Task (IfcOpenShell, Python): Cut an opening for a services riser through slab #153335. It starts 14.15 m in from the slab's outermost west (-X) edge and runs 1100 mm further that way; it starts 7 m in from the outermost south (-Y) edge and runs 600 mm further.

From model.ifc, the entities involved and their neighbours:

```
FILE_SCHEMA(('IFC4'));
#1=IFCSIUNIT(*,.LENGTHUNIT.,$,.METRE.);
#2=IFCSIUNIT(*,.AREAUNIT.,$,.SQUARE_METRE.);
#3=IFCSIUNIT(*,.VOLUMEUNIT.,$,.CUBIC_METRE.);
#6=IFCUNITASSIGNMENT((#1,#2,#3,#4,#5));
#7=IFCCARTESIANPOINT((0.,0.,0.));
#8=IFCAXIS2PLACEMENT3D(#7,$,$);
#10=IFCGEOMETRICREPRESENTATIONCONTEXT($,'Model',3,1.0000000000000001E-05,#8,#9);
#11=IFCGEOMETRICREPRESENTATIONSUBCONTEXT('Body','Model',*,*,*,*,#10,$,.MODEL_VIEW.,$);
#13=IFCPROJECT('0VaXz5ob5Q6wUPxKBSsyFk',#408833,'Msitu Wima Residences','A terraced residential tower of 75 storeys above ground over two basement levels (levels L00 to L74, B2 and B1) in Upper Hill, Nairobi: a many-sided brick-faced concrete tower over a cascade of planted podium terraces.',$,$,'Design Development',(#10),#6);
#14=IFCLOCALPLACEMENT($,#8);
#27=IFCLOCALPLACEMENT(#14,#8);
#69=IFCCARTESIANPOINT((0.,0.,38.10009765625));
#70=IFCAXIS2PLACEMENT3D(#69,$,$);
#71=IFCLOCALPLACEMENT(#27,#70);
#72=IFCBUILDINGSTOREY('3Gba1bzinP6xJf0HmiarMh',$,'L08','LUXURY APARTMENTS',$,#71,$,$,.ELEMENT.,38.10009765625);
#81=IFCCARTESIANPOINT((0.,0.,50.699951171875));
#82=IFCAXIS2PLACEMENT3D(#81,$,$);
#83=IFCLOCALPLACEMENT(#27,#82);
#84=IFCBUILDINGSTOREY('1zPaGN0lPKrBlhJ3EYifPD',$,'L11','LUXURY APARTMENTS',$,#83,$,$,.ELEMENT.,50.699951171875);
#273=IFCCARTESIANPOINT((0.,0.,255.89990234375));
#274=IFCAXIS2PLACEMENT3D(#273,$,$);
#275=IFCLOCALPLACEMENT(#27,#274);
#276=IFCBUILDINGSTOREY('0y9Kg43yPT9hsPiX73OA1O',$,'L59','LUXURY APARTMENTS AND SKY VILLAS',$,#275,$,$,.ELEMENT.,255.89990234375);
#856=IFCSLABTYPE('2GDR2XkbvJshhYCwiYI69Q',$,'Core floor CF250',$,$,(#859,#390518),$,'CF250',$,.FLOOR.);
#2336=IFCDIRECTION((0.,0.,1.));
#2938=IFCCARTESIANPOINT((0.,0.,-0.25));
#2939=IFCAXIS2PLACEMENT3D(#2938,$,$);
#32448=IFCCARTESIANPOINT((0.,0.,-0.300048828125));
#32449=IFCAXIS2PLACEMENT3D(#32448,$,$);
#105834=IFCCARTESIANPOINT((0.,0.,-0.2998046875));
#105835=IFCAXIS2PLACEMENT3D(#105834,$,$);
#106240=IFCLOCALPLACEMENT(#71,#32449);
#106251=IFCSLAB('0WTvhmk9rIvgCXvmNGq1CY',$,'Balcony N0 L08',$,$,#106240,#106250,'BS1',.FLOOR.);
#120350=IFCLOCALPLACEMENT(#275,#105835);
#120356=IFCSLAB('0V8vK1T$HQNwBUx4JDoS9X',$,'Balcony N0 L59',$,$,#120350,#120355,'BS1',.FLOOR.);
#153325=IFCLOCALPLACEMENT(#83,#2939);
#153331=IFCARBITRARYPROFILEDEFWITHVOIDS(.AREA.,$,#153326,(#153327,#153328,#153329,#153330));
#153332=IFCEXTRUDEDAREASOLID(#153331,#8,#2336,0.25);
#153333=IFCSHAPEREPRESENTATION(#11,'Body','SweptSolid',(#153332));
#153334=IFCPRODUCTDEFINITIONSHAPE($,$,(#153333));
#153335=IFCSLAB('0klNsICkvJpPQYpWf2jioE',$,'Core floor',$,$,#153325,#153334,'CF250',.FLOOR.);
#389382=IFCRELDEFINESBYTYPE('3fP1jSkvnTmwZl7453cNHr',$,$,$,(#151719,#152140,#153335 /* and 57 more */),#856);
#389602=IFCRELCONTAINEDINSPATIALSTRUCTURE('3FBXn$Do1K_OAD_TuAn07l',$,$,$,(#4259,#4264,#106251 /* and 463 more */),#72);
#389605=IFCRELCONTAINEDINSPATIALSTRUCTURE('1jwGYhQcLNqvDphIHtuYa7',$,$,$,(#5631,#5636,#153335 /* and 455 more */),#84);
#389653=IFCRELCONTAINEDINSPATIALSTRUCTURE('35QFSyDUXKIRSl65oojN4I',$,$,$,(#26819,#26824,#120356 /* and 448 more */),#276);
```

```python
import numpy as np
import ifcopenshell
import ifcopenshell.api.feature
import ifcopenshell.api.geometry
import ifcopenshell.api.root
import ifcopenshell.geom
import ifcopenshell.util.placement
import ifcopenshell.util.representation
import ifcopenshell.util.shape
import ifcopenshell.util.unit

model = ifcopenshell.open("model.ifc")
unit_scale = ifcopenshell.util.unit.calculate_unit_scale(model)
settings = ifcopenshell.geom.settings()


def volume(element):
    """Net volume in cubic metres, openings subtracted."""
    shape = ifcopenshell.geom.create_shape(settings, element)
    return ifcopenshell.util.shape.get_volume(shape.geometry)


slab = model.by_id(153335)
before = volume(slab)

# Extent in the slab's own axes, in metres. The edges named are its -X and -Y sides.
slab_shape = ifcopenshell.geom.create_shape(settings, slab)
vertices = ifcopenshell.util.shape.get_vertices(slab_shape.geometry)
x_min, y_min, bottom = vertices.min(axis=0)
top = vertices[:, 2].max()

opening = ifcopenshell.api.root.create_entity(model, ifc_class="IfcOpeningElement", name="Services riser opening", predefined_type="OPENING")
context = ifcopenshell.util.representation.get_context(model, "Model", "Body", "MODEL_VIEW")
width, depth = 1.1, 0.6
outline = [(0.0, 0.0), (width, 0.0), (width, depth), (0.0, depth), (0.0, 0.0)]
# Overshoot both faces by 50 mm so the cut is clean.
shape = ifcopenshell.api.geometry.add_slab_representation(
    model, context=context, depth=top - bottom + 0.1, polyline=outline
)
ifcopenshell.api.geometry.assign_representation(model, product=opening, representation=shape)

matrix = ifcopenshell.util.placement.get_local_placement(slab.ObjectPlacement)
matrix[:, 3] = matrix @ np.append(np.array([x_min + 14.15, y_min + 7, bottom - 0.05]) / unit_scale, 1.0)
ifcopenshell.api.geometry.edit_object_placement(model, product=opening, matrix=matrix, is_si=False)
ifcopenshell.api.feature.add_feature(model, feature=opening, element=slab)

after = volume(slab)

print(f"slab volume {before:.3f} -> {after:.3f} m3")

model.write("model_v2.ifc")
```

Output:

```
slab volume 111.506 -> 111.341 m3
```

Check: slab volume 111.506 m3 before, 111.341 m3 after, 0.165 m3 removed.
